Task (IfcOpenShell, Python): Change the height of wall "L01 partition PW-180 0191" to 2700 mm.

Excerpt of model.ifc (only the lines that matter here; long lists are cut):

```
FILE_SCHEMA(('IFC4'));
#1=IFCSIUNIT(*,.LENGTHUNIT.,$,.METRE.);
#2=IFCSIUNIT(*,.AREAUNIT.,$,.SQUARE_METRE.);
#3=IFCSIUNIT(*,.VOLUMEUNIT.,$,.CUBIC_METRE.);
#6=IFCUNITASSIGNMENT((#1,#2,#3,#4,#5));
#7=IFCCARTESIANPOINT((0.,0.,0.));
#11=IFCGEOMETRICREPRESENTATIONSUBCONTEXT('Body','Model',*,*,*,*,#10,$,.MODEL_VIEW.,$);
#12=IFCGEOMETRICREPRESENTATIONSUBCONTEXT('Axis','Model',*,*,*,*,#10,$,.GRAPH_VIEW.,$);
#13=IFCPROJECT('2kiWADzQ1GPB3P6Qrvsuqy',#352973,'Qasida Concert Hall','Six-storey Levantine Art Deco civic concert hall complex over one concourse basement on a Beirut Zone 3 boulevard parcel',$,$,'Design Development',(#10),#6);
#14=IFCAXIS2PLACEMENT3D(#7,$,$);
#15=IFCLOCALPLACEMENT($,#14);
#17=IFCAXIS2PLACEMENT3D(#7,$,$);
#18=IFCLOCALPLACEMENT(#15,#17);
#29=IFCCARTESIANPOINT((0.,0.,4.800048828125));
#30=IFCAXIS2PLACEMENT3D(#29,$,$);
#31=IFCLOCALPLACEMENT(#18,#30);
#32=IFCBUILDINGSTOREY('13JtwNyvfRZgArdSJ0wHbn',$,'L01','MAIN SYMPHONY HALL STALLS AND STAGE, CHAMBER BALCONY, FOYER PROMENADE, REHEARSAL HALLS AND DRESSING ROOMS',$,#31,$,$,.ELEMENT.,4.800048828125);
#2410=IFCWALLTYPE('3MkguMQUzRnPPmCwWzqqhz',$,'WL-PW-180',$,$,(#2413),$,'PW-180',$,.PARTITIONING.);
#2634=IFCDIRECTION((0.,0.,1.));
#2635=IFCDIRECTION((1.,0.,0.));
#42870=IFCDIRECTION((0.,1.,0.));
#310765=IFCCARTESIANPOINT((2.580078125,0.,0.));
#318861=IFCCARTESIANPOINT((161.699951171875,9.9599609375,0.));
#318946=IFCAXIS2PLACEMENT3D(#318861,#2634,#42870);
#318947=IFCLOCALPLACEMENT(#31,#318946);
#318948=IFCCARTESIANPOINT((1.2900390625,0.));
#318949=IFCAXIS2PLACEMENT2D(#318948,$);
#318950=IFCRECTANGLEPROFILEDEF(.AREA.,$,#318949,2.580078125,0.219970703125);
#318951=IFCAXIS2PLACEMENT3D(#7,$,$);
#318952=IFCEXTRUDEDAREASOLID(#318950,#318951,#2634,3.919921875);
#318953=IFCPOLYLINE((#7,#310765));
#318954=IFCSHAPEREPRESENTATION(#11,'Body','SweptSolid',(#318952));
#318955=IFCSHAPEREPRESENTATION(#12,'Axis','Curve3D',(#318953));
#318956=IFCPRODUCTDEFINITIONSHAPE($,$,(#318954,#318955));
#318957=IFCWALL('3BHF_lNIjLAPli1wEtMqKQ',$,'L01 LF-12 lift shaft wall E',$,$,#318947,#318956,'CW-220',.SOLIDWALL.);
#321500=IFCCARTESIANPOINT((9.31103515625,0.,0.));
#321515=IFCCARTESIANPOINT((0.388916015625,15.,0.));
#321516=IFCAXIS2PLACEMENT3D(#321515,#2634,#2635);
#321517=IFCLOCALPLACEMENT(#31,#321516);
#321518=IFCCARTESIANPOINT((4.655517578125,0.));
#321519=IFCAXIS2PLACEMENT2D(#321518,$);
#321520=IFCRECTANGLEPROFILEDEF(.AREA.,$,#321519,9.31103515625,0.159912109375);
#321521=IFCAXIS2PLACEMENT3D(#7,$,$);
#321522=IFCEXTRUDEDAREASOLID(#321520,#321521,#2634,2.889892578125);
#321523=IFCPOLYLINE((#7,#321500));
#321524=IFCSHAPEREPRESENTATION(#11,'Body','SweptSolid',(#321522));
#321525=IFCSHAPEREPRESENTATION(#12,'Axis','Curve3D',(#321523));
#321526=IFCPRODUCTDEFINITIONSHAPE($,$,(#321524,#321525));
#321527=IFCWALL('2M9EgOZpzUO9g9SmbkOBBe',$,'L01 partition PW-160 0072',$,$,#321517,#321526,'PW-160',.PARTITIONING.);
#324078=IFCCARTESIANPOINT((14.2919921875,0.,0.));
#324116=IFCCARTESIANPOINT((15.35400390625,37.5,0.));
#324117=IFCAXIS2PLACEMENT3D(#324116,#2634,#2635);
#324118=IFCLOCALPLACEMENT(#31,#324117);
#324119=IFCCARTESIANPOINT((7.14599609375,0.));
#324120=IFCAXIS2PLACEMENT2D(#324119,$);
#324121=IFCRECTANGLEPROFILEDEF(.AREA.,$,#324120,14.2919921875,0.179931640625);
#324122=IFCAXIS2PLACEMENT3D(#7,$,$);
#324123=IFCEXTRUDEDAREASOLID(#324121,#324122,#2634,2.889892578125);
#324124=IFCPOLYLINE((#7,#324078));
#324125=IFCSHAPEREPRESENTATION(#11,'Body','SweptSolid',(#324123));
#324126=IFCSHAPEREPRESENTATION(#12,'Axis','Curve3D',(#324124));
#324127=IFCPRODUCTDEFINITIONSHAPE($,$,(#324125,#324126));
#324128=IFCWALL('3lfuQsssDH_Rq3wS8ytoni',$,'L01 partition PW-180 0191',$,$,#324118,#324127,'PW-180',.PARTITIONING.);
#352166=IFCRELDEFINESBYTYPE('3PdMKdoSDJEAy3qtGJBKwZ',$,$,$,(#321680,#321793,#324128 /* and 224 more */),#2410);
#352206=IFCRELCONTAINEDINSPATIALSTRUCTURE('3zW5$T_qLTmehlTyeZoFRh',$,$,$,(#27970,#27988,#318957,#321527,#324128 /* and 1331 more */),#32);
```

```python
import ifcopenshell
import ifcopenshell.geom
import ifcopenshell.util.representation
import ifcopenshell.util.shape

model = ifcopenshell.open("model.ifc")
settings = ifcopenshell.geom.settings()


def volume(element):
    """Net volume in cubic metres, openings subtracted."""
    shape = ifcopenshell.geom.create_shape(settings, element)
    return ifcopenshell.util.shape.get_volume(shape.geometry)


wall = model.by_guid("3lfuQsssDH_Rq3wS8ytoni")
before = volume(wall)

body = ifcopenshell.util.representation.get_representation(wall, "Model", "Body")
solid = body.Items[0]
old_height = solid.Depth
solid.Depth = 2.7
after = volume(wall)

print(f"height {old_height:g} -> {solid.Depth:g}, volume {before:.3f} -> {after:.3f} m3")

model.write("model_v2.ifc")
```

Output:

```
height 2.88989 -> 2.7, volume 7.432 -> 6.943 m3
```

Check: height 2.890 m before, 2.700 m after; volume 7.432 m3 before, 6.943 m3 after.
